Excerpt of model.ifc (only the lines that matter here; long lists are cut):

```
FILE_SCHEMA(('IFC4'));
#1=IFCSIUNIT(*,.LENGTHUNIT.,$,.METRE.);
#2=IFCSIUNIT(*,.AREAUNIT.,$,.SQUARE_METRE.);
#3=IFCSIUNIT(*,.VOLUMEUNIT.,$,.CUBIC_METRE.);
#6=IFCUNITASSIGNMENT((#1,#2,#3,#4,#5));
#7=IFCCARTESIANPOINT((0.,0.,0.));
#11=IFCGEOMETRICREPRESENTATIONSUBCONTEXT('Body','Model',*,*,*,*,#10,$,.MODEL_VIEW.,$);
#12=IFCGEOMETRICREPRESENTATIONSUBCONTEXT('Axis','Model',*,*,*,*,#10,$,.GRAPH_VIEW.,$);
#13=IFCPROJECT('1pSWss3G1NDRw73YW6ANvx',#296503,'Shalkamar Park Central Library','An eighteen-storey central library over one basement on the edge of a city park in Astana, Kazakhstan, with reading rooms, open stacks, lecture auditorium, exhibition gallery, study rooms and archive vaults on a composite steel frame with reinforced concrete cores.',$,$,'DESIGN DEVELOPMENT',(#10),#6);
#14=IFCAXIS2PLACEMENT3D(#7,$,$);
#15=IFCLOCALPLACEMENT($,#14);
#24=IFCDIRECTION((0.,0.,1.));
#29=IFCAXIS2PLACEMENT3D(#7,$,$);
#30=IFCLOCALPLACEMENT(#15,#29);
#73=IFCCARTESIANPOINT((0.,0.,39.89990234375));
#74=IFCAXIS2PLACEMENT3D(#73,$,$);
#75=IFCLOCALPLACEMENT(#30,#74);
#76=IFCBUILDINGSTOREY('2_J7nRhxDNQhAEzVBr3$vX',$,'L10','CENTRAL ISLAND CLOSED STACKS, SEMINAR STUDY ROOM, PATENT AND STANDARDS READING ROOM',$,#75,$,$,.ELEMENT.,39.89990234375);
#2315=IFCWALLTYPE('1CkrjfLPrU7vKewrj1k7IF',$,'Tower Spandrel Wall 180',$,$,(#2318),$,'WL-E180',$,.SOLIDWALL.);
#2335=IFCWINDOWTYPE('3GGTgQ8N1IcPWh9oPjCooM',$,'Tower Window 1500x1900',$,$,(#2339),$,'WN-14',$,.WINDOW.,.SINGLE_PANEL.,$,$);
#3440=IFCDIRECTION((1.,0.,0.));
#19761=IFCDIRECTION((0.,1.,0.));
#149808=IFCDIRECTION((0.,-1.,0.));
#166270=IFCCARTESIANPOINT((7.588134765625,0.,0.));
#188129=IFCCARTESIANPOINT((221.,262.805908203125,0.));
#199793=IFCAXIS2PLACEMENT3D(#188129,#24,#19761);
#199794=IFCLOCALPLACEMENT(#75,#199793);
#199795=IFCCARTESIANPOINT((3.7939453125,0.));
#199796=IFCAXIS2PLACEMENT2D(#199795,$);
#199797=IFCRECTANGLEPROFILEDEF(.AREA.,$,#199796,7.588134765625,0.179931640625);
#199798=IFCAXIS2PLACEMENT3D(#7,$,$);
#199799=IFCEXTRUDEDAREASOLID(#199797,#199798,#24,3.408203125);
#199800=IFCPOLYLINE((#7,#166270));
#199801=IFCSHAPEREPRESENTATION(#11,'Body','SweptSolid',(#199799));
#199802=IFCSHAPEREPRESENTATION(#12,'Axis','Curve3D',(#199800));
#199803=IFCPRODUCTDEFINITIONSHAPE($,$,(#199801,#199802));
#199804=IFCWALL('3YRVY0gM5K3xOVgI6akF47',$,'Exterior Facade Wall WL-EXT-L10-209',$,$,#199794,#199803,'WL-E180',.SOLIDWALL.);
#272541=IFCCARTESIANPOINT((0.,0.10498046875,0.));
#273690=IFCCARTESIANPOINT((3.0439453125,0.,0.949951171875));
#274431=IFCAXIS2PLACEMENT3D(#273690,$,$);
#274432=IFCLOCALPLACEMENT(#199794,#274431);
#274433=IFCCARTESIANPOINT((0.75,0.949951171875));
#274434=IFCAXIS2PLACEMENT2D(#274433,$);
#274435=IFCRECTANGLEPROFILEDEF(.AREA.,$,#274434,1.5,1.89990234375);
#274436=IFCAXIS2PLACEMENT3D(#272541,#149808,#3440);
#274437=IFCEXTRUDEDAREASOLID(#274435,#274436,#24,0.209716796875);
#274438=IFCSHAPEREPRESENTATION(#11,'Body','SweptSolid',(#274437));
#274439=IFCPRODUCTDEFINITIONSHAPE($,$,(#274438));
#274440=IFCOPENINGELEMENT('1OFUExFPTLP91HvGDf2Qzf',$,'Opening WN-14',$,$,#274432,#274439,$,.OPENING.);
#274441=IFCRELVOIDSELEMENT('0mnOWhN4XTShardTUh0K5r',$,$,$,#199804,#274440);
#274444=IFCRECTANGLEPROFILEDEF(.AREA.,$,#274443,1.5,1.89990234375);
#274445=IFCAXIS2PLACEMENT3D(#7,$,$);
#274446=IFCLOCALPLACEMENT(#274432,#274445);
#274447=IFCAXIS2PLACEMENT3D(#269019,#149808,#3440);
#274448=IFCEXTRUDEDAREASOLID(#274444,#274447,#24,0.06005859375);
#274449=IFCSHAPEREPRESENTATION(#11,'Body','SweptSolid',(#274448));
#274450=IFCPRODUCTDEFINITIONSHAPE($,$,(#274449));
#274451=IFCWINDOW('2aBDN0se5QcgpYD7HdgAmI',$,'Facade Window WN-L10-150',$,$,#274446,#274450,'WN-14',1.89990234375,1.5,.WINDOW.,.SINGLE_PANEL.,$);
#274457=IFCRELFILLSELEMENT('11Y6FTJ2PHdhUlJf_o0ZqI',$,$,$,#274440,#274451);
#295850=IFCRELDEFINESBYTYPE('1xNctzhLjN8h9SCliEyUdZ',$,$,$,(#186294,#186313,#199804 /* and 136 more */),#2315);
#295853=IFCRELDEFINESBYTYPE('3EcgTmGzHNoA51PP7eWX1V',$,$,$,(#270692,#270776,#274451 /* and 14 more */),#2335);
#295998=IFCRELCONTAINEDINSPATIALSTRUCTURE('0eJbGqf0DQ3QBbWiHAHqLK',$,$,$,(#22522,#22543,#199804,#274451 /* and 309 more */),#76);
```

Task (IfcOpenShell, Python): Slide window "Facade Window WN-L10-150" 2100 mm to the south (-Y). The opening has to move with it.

```python
import ifcopenshell
import ifcopenshell.api.geometry
import ifcopenshell.util.placement

model = ifcopenshell.open("model.ifc")

window = model.by_guid("2aBDN0se5QcgpYD7HdgAmI")
opening = window.FillsVoids[0].RelatingOpeningElement
wall = opening.VoidsElements[0].RelatingBuildingElement

wall_matrix = ifcopenshell.util.placement.get_local_placement(wall.ObjectPlacement)
shift = wall_matrix[:3, 0] * -2.1
before = ifcopenshell.util.placement.get_local_placement(window.ObjectPlacement)[:3, 3].copy()

# The window is placed relative to its opening, so it follows when the opening moves.
matrix = ifcopenshell.util.placement.get_local_placement(opening.ObjectPlacement)
matrix[:3, 3] += shift
ifcopenshell.api.geometry.edit_object_placement(
    model, product=opening, matrix=matrix, is_si=False, should_transform_children=True
)

after = ifcopenshell.util.placement.get_local_placement(window.ObjectPlacement)[:3, 3]
print("window moved by", (after - before).round(3) + 0.0)

model.write("model_rev.ifc")
```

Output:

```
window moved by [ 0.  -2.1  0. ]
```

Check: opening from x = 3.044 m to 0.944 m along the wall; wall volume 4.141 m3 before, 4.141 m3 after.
